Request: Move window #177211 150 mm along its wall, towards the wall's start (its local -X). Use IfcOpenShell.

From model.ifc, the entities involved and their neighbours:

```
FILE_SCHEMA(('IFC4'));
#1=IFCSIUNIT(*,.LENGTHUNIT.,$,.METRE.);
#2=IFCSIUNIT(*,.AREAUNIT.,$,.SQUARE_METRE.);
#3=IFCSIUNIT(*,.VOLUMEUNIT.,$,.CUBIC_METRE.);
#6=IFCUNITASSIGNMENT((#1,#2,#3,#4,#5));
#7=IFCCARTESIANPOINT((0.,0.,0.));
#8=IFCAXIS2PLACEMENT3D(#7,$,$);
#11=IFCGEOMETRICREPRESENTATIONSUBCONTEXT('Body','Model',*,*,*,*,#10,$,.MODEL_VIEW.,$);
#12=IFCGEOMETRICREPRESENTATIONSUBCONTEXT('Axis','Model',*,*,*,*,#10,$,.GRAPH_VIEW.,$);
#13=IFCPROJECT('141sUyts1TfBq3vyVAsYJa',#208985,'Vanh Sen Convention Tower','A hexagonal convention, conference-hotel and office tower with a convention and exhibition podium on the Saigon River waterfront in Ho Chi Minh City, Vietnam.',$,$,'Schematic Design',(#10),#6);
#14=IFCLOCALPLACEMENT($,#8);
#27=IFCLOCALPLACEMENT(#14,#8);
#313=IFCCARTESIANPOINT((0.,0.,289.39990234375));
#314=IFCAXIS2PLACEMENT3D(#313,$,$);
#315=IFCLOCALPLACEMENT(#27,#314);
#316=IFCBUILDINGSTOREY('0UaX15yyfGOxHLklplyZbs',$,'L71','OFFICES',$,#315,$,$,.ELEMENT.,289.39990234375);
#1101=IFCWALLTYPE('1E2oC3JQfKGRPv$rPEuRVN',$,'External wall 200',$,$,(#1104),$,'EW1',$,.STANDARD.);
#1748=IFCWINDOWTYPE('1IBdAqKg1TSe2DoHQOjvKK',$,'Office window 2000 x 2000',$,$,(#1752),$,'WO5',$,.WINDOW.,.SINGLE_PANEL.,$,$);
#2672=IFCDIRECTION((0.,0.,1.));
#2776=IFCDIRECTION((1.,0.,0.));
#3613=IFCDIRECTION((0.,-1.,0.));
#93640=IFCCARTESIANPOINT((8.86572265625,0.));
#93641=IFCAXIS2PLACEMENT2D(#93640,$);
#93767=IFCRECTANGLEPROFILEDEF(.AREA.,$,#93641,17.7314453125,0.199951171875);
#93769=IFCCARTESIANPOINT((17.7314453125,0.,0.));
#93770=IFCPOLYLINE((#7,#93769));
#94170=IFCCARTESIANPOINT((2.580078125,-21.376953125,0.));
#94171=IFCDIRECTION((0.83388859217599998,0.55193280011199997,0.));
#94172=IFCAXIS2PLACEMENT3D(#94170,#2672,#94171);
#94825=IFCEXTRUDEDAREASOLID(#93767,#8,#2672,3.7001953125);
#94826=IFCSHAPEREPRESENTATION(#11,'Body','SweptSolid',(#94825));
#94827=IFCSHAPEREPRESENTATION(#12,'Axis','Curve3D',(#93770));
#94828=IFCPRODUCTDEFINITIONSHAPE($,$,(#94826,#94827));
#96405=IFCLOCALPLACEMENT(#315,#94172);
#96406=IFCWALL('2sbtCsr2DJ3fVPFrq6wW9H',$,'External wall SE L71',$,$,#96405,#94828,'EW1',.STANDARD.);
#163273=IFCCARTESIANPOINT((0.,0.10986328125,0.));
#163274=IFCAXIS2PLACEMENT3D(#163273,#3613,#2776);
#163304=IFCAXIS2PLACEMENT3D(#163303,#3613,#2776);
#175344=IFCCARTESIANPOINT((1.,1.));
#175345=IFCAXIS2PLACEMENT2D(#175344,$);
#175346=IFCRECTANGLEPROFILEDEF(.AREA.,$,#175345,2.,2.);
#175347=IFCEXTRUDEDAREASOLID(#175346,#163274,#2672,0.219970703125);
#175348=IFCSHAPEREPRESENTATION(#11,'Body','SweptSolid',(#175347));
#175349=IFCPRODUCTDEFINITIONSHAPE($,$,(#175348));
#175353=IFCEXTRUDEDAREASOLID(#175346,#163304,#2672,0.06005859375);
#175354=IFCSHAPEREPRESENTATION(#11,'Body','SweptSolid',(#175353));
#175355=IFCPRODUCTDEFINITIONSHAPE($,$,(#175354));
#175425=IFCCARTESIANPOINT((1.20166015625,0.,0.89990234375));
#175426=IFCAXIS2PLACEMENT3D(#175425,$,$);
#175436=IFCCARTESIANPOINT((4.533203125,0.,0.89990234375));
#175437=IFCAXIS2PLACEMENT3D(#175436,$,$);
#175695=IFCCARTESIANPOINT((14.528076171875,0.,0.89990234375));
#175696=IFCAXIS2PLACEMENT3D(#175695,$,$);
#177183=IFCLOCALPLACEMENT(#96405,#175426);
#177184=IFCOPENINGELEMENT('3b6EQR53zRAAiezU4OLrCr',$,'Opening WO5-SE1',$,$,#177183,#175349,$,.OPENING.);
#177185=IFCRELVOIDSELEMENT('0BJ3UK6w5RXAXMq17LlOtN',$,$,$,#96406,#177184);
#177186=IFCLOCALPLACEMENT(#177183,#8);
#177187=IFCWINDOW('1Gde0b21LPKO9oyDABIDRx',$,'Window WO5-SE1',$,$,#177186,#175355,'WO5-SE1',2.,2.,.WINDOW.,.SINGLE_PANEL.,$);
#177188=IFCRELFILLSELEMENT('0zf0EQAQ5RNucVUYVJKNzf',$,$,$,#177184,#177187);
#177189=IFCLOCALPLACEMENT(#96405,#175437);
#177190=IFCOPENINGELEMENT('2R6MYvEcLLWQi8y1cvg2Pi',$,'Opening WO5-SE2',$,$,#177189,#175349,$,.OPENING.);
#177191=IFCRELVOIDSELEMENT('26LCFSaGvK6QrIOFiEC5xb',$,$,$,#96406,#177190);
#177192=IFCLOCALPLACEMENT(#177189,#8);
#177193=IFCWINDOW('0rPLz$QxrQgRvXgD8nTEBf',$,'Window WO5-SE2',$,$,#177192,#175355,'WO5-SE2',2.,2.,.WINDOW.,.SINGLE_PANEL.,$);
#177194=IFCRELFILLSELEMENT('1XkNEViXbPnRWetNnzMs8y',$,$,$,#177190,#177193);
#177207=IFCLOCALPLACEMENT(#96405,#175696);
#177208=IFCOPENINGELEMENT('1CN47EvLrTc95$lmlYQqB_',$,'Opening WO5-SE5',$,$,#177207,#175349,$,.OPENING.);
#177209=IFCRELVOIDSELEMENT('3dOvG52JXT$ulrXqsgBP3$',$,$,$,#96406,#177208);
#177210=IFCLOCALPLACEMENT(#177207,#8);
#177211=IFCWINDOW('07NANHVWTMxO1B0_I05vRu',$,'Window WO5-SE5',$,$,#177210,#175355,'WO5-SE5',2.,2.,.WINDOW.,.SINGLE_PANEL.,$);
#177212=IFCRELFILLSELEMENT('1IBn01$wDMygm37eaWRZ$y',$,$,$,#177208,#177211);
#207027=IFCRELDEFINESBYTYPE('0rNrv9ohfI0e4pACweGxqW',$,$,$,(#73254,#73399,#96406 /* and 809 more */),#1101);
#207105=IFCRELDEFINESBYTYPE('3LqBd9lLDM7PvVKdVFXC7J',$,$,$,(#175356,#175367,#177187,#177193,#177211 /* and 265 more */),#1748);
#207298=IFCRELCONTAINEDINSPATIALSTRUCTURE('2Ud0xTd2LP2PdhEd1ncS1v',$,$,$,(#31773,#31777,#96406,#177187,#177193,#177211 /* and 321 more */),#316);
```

```python
import ifcopenshell
import ifcopenshell.api.geometry
import ifcopenshell.util.placement
import ifcopenshell.util.unit

model = ifcopenshell.open("model.ifc")
unit_scale = ifcopenshell.util.unit.calculate_unit_scale(model)

window = model.by_id(177211)
opening = window.FillsVoids[0].RelatingOpeningElement
wall = opening.VoidsElements[0].RelatingBuildingElement

wall_matrix = ifcopenshell.util.placement.get_local_placement(wall.ObjectPlacement)
shift = wall_matrix[:3, 0] * -0.15 / unit_scale
before = ifcopenshell.util.placement.get_local_placement(window.ObjectPlacement)[:3, 3].copy()

# The window is placed relative to its opening, so it follows when the opening moves.
matrix = ifcopenshell.util.placement.get_local_placement(opening.ObjectPlacement)
matrix[:3, 3] += shift
ifcopenshell.api.geometry.edit_object_placement(
    model, product=opening, matrix=matrix, is_si=False, should_transform_children=True
)

after = ifcopenshell.util.placement.get_local_placement(window.ObjectPlacement)[:3, 3]
print("window moved by", (after - before).round(3) + 0.0)

model.write("model_edited.ifc")
```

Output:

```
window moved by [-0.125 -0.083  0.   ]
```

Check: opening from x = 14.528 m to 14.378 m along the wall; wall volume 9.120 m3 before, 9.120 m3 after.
